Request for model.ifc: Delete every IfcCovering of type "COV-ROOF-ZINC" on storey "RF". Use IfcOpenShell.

First a look at what the model holds.

```python
import ifcopenshell
import ifcopenshell.util.element

model = ifcopenshell.open("model.ifc")
print(model.schema)
storey = next(s for s in model.by_type("IfcBuildingStorey") if s.Name == "RF")
coverings = [e for e in ifcopenshell.util.element.get_decomposition(storey) if e.is_a("IfcCovering")]
seen = {}
for e in coverings:
    element_type = ifcopenshell.util.element.get_type(e)
    name = element_type.Name if element_type not in (None, e) else None
    seen[name] = seen.get(name, 0) + 1
for name, count in sorted(seen.items(), key=str):
    print(count, "x", name)
```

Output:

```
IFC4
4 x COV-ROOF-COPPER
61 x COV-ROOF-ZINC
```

```python
import ifcopenshell
import ifcopenshell.api.root
import ifcopenshell.util.element

model = ifcopenshell.open("model.ifc")

storey = next(s for s in model.by_type("IfcBuildingStorey") if s.Name == "RF")
coverings = [e for e in ifcopenshell.util.element.get_decomposition(storey) if e.is_a("IfcCovering")]
targets = [e for e in coverings if (t := ifcopenshell.util.element.get_type(e)) not in (None, e) and t.Name == "COV-ROOF-ZINC"]

for e in targets:
    ifcopenshell.api.root.remove_product(model, product=e)
print(len(targets), "removed")

model.write("model_v2.ifc")
```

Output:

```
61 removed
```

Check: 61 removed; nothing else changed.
